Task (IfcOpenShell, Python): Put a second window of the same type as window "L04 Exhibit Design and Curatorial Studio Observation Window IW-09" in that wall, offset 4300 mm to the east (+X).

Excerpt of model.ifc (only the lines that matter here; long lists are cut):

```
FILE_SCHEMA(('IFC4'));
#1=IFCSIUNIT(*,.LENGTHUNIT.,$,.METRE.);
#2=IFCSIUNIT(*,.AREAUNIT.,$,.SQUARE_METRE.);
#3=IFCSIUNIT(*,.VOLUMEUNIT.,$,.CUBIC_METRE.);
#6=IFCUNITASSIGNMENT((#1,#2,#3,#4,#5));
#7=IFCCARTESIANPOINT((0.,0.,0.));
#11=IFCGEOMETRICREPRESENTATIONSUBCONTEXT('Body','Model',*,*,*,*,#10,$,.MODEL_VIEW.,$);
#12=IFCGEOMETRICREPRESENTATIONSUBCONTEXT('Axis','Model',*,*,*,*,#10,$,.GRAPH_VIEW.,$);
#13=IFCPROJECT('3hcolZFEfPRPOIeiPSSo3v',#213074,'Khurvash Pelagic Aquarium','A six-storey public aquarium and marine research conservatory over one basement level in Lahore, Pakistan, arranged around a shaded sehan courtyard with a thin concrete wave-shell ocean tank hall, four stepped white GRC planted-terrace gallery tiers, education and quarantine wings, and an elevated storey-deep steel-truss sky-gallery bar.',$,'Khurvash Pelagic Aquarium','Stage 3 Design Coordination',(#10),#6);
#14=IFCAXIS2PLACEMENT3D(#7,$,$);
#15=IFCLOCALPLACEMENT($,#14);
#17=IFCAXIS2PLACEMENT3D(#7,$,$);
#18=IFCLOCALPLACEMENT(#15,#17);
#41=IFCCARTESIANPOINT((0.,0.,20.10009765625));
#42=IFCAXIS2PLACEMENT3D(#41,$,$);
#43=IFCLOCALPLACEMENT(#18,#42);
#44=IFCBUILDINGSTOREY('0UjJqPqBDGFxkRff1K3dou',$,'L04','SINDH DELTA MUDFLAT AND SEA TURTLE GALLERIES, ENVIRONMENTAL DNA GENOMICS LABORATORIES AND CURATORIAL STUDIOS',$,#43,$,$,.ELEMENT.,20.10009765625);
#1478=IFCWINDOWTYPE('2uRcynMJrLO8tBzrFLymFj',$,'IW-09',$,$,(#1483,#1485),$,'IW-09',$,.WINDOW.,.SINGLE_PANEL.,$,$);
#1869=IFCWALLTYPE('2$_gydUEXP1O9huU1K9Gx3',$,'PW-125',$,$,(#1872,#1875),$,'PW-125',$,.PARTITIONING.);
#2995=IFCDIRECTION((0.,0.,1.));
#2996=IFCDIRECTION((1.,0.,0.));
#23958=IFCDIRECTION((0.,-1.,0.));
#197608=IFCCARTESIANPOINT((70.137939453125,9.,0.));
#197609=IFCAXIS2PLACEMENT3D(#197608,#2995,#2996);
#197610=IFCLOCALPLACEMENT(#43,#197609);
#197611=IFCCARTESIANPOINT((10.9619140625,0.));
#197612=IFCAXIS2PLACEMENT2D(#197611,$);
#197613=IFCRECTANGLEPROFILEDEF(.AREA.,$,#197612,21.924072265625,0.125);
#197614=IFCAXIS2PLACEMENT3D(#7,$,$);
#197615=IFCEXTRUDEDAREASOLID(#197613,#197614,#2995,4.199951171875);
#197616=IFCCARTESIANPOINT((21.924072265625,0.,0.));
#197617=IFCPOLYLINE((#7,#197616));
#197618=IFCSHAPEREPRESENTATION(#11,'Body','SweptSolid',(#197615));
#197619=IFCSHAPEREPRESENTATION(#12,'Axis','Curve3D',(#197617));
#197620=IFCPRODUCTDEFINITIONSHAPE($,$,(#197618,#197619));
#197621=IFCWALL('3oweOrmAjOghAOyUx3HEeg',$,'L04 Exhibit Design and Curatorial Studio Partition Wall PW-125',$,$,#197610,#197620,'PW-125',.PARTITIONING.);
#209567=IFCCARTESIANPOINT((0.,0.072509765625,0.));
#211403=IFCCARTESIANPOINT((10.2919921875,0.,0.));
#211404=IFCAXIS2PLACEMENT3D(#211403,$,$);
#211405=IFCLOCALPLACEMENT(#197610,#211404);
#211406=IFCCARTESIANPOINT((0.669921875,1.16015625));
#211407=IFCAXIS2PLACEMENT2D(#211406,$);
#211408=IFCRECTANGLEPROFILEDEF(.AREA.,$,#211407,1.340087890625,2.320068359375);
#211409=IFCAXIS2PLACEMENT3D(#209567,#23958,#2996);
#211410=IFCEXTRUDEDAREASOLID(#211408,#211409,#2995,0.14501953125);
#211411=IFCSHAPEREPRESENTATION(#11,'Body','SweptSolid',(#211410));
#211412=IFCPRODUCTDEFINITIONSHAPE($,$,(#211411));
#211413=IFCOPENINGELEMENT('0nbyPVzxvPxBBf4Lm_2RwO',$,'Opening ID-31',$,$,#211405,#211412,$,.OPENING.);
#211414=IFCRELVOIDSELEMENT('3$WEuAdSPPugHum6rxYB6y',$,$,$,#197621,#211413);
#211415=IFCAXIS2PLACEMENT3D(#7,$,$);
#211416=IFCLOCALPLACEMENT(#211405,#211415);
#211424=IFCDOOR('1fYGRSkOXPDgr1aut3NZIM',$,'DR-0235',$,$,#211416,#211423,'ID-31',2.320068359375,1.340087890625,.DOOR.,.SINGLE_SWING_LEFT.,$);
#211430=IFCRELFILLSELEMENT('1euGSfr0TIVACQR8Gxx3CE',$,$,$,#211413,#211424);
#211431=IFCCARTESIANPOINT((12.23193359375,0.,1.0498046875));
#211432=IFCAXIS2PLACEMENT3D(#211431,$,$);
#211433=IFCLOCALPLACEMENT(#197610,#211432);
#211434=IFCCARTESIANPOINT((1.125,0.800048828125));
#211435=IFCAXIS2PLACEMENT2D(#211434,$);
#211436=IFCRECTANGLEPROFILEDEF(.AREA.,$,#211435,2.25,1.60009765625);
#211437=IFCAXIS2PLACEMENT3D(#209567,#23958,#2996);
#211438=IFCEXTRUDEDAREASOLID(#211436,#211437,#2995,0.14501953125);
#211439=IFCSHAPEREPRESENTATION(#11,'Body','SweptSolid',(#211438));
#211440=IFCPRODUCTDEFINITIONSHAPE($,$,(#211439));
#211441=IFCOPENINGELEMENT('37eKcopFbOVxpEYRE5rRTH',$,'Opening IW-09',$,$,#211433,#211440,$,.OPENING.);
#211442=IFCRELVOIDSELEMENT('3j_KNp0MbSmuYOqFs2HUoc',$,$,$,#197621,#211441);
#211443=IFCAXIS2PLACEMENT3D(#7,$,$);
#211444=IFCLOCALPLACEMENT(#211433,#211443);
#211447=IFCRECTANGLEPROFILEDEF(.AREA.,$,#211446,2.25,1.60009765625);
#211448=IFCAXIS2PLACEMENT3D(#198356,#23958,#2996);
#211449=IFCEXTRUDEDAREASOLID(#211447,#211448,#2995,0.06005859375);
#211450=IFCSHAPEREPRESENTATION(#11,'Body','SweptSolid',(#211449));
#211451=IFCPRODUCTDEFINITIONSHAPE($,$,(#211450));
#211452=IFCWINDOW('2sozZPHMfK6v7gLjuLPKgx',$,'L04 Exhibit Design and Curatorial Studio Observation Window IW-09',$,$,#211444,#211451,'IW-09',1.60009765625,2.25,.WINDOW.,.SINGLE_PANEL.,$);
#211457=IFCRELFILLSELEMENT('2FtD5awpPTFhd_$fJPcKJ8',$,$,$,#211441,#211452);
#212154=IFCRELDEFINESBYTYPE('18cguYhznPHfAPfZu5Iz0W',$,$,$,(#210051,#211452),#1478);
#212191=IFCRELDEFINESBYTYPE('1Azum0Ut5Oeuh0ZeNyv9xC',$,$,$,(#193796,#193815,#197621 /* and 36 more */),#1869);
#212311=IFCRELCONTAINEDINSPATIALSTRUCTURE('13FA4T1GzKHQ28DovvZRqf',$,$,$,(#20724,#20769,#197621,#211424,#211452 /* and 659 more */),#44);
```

```python
import ifcopenshell
import ifcopenshell.api.feature
import ifcopenshell.api.geometry
import ifcopenshell.api.root
import ifcopenshell.geom
import ifcopenshell.util.element
import ifcopenshell.util.placement
import ifcopenshell.util.shape

model = ifcopenshell.open("model.ifc")
settings = ifcopenshell.geom.settings()


def volume(element):
    """Net volume in cubic metres, openings subtracted."""
    shape = ifcopenshell.geom.create_shape(settings, element)
    return ifcopenshell.util.shape.get_volume(shape.geometry)


window = model.by_guid("2sozZPHMfK6v7gLjuLPKgx")
opening = window.FillsVoids[0].RelatingOpeningElement
wall = opening.VoidsElements[0].RelatingBuildingElement
before = volume(wall)
shift = ifcopenshell.util.placement.get_local_placement(wall.ObjectPlacement)[:3, 0] * 4.3

# copy_class copies the void relationship, type, container and properties, but no geometry.
new_opening = ifcopenshell.api.root.copy_class(model, product=opening)
new_opening.Representation = ifcopenshell.util.element.copy_deep(
    model, opening.Representation, exclude=["IfcGeometricRepresentationContext", "IfcRepresentationMap"]
)
new_window = ifcopenshell.api.root.copy_class(model, product=window)
new_window.Representation = ifcopenshell.util.element.copy_deep(
    model, window.Representation, exclude=["IfcGeometricRepresentationContext", "IfcRepresentationMap"]
)
new_window.Tag = None
ifcopenshell.api.feature.add_filling(model, opening=new_opening, element=new_window)

for old, new in ((opening, new_opening), (window, new_window)):
    matrix = ifcopenshell.util.placement.get_local_placement(old.ObjectPlacement)
    matrix[:3, 3] += shift
    ifcopenshell.api.geometry.edit_object_placement(model, product=new, matrix=matrix, is_si=False)

after = volume(wall)

print(f"wall volume {before:.3f} -> {after:.3f} m3")

model.write("model_v2.ifc")
```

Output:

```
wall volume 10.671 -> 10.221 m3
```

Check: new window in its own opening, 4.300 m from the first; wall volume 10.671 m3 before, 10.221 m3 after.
